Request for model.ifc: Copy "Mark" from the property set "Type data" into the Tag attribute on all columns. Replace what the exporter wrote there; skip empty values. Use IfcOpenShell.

First a look at what the model holds.

```python
import ifcopenshell
import ifcopenshell.util.element

model = ifcopenshell.open("model.ifc")
print(model.schema)
columns = model.by_type("IfcColumn")
print(len(columns), "columns")
for e in columns[:8]:
    source = ifcopenshell.util.element.get_pset(e, "Type data", "Mark")
    target = e.Tag
    print(e.id(), repr(source), repr(target), sep=" | ")
```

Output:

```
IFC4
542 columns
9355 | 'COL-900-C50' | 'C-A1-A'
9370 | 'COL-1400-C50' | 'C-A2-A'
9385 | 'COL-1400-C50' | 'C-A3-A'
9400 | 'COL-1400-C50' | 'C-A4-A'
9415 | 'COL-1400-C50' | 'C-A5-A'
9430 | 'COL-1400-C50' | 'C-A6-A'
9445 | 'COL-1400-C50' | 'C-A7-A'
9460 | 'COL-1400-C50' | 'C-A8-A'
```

```python
import ifcopenshell
import ifcopenshell.util.element

model = ifcopenshell.open("model.ifc")

count = 0
for e in model.by_type("IfcColumn"):
    value = ifcopenshell.util.element.get_pset(e, "Type data", "Mark")
    current = e.Tag
    if not value or not value.strip() or current == value:
        continue
    e.Tag = value
    count += 1

print(count, "columns updated")

model.write("model_updated.ifc")
```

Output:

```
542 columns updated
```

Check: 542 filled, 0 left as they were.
